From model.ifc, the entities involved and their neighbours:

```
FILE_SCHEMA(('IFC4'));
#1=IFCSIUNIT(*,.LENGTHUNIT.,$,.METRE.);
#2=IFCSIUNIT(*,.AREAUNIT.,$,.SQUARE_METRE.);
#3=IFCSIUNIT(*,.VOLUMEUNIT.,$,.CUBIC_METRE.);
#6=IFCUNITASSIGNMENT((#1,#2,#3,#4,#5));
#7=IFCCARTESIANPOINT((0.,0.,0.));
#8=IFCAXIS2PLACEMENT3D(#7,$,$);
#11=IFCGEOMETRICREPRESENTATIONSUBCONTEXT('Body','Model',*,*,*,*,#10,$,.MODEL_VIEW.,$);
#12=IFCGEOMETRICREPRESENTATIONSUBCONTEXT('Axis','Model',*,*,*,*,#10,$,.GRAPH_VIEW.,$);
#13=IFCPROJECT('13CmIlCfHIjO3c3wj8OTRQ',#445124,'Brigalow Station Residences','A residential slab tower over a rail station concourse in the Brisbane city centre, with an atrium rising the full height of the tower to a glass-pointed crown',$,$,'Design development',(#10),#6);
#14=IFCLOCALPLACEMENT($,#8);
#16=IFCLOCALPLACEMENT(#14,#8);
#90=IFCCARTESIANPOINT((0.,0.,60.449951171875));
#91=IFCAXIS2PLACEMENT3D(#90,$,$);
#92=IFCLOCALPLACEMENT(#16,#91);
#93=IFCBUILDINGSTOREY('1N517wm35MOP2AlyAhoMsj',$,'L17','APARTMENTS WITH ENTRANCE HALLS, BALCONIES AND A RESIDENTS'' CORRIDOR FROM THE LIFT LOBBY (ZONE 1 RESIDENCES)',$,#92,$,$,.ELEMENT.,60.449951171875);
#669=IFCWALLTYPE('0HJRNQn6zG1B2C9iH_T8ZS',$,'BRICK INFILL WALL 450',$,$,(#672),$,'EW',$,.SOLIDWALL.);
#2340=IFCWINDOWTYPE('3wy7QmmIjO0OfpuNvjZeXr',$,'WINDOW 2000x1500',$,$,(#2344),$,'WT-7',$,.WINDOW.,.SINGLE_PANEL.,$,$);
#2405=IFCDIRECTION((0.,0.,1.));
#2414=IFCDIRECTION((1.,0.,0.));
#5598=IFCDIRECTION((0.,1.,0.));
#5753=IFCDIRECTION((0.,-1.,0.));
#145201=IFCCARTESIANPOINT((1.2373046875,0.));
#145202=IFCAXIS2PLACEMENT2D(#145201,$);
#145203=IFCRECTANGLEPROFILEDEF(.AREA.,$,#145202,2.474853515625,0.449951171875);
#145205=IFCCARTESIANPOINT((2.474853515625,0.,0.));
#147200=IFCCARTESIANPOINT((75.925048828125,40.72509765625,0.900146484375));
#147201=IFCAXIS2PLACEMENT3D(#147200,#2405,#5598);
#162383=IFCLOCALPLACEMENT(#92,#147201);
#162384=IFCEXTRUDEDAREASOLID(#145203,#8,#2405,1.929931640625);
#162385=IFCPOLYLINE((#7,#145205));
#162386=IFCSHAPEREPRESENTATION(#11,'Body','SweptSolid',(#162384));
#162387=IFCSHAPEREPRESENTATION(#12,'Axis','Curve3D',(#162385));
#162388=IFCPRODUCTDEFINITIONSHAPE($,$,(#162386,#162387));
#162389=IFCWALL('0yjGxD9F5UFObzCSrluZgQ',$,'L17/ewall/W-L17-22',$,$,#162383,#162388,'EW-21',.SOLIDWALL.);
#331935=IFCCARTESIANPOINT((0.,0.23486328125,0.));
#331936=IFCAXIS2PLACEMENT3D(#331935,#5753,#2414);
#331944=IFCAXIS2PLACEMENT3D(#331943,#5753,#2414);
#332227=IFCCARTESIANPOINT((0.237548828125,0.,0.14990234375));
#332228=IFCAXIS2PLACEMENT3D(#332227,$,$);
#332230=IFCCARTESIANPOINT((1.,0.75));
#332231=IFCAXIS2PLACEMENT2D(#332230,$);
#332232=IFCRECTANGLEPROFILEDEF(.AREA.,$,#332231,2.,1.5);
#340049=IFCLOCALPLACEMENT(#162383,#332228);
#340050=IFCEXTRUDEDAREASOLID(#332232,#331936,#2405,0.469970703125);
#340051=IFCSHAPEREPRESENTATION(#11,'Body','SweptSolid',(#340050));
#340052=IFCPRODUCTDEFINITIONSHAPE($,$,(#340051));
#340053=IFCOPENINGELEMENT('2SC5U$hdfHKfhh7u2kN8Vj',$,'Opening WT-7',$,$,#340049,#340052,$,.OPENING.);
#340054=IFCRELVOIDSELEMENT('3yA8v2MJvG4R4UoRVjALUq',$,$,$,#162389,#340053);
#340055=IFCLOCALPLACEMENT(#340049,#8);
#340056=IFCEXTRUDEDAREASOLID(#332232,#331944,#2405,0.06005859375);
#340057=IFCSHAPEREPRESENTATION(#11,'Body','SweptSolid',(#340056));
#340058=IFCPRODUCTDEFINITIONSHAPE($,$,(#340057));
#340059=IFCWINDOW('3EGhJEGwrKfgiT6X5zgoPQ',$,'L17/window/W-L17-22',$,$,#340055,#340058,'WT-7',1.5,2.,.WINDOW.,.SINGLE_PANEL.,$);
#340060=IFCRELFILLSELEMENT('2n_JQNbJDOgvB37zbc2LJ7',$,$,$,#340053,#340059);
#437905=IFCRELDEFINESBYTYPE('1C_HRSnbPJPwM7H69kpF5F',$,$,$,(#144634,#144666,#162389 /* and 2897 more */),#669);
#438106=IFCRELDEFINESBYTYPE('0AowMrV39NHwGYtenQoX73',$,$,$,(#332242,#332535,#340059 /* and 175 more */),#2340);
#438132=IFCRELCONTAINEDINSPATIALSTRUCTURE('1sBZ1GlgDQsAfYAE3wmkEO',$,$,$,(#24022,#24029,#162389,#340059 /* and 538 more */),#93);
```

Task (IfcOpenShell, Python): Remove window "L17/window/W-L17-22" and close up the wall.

```python
import ifcopenshell
import ifcopenshell.api.feature
import ifcopenshell.api.root
import ifcopenshell.geom
import ifcopenshell.util.shape

model = ifcopenshell.open("model.ifc")
settings = ifcopenshell.geom.settings()


def volume(element):
    """Net volume in cubic metres, openings subtracted."""
    shape = ifcopenshell.geom.create_shape(settings, element)
    return ifcopenshell.util.shape.get_volume(shape.geometry)


window = model.by_guid("3EGhJEGwrKfgiT6X5zgoPQ")
opening = window.FillsVoids[0].RelatingOpeningElement
wall = opening.VoidsElements[0].RelatingBuildingElement
before = volume(wall)

ifcopenshell.api.root.remove_product(model, product=window)
ifcopenshell.api.feature.remove_feature(model, feature=opening)

after = volume(wall)

print(f"wall volume {before:.3f} -> {after:.3f} m3")

model.write("model_rev.ifc")
```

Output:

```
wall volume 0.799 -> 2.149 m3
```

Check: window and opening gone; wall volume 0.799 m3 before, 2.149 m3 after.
